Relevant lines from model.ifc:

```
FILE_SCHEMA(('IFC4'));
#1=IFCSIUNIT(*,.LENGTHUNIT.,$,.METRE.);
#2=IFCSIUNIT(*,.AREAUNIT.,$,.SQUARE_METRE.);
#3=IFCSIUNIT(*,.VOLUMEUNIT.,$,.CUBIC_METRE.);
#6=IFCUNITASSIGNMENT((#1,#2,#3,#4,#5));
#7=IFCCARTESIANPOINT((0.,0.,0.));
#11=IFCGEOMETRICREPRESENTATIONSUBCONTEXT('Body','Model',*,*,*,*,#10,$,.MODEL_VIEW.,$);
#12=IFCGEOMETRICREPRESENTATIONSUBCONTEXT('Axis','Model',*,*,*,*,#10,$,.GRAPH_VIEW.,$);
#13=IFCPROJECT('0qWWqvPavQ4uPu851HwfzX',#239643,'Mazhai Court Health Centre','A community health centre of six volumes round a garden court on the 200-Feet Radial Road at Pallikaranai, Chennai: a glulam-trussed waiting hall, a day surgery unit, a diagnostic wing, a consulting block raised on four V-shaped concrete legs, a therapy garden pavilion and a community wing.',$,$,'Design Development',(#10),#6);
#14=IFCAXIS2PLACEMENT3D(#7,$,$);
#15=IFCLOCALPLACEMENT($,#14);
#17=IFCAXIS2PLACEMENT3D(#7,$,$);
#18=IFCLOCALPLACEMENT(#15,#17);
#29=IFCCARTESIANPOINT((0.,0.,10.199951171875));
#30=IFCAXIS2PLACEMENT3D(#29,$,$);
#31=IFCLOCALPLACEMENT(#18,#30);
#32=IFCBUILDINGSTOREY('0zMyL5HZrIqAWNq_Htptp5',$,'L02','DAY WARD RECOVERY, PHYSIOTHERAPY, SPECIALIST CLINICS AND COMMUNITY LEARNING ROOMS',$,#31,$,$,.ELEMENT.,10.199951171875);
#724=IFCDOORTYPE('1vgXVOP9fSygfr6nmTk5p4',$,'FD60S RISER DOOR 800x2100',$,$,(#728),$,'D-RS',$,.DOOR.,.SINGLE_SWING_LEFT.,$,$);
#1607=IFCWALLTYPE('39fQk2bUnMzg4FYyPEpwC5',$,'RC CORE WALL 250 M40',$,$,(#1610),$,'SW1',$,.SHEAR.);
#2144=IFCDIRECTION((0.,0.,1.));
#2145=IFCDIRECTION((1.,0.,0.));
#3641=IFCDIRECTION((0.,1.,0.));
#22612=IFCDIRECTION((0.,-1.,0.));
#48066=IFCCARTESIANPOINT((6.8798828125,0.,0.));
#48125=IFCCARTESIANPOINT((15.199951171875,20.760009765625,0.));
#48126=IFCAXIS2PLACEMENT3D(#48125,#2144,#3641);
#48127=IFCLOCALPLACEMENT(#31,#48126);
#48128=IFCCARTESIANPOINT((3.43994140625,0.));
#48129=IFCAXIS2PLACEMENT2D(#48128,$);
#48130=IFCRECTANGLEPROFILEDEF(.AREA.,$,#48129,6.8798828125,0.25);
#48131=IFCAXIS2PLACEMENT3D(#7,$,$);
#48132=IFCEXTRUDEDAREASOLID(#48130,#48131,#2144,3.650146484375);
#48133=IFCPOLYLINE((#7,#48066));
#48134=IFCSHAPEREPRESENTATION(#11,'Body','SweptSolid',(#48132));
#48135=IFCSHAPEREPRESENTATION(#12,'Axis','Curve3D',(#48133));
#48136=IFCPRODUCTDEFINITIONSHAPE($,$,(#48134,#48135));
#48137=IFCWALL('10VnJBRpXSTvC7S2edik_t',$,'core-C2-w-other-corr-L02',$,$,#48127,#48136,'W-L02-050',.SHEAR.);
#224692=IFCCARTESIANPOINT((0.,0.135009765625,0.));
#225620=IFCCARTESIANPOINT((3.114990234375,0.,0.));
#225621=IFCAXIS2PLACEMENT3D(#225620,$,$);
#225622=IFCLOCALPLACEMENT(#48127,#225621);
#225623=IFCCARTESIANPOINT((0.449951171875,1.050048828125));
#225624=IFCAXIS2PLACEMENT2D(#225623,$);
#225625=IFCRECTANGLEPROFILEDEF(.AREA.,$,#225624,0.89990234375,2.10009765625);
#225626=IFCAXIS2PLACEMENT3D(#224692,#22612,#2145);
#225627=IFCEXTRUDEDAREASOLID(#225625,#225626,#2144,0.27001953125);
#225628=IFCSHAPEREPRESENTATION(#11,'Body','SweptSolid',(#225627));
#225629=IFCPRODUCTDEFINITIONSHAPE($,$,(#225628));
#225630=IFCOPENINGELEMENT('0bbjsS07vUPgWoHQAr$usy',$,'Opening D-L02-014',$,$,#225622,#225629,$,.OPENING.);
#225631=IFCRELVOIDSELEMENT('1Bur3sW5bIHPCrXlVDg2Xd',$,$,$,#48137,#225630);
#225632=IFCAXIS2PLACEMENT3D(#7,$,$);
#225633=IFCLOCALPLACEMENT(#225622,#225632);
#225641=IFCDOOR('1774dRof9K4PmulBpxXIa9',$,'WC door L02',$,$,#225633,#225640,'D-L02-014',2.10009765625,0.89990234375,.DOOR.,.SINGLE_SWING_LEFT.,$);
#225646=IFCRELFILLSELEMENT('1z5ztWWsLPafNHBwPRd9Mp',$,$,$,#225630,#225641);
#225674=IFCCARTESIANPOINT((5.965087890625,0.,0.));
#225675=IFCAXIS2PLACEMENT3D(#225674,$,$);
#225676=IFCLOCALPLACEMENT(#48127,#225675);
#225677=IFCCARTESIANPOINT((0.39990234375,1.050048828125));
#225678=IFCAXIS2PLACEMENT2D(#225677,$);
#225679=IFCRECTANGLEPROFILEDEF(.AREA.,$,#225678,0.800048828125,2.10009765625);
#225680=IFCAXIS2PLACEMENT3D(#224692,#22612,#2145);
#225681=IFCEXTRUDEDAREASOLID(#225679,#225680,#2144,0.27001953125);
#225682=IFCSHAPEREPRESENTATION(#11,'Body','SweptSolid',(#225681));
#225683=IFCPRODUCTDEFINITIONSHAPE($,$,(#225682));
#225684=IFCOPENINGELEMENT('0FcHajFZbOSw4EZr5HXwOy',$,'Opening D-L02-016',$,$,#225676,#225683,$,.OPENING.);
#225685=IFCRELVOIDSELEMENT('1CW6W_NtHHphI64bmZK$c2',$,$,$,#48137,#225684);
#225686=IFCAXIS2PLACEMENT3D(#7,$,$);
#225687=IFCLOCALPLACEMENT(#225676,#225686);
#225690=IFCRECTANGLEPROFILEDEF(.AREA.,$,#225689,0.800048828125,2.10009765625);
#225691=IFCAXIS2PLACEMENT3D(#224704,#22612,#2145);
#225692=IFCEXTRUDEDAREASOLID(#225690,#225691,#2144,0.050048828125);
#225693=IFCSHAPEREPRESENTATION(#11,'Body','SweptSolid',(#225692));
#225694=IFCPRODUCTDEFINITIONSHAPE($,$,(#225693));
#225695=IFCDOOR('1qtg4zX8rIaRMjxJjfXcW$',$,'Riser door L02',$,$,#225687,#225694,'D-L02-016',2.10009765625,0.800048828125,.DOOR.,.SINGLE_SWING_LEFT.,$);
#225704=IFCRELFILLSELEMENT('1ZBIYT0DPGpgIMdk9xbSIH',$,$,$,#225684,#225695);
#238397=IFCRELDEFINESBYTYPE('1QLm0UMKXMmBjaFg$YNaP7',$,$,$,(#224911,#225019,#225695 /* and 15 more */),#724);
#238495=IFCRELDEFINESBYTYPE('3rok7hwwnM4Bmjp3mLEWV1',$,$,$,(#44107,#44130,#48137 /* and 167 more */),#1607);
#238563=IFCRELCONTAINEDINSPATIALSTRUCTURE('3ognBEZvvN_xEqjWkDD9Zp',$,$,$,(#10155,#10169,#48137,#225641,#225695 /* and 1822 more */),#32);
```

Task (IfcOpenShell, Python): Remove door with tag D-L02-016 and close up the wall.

```python
import ifcopenshell
import ifcopenshell.api.feature
import ifcopenshell.api.root
import ifcopenshell.geom
import ifcopenshell.util.shape

model = ifcopenshell.open("model.ifc")
settings = ifcopenshell.geom.settings()


def volume(element):
    """Net volume in cubic metres, openings subtracted."""
    shape = ifcopenshell.geom.create_shape(settings, element)
    return ifcopenshell.util.shape.get_volume(shape.geometry)


door = model.by_id(225695)
opening = door.FillsVoids[0].RelatingOpeningElement
wall = opening.VoidsElements[0].RelatingBuildingElement
before = volume(wall)

ifcopenshell.api.root.remove_product(model, product=door)
ifcopenshell.api.feature.remove_feature(model, feature=opening)

after = volume(wall)

print(f"wall volume {before:.3f} -> {after:.3f} m3")

model.write("model_v2.ifc")
```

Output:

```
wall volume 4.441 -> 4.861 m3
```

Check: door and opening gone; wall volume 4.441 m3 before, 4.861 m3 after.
